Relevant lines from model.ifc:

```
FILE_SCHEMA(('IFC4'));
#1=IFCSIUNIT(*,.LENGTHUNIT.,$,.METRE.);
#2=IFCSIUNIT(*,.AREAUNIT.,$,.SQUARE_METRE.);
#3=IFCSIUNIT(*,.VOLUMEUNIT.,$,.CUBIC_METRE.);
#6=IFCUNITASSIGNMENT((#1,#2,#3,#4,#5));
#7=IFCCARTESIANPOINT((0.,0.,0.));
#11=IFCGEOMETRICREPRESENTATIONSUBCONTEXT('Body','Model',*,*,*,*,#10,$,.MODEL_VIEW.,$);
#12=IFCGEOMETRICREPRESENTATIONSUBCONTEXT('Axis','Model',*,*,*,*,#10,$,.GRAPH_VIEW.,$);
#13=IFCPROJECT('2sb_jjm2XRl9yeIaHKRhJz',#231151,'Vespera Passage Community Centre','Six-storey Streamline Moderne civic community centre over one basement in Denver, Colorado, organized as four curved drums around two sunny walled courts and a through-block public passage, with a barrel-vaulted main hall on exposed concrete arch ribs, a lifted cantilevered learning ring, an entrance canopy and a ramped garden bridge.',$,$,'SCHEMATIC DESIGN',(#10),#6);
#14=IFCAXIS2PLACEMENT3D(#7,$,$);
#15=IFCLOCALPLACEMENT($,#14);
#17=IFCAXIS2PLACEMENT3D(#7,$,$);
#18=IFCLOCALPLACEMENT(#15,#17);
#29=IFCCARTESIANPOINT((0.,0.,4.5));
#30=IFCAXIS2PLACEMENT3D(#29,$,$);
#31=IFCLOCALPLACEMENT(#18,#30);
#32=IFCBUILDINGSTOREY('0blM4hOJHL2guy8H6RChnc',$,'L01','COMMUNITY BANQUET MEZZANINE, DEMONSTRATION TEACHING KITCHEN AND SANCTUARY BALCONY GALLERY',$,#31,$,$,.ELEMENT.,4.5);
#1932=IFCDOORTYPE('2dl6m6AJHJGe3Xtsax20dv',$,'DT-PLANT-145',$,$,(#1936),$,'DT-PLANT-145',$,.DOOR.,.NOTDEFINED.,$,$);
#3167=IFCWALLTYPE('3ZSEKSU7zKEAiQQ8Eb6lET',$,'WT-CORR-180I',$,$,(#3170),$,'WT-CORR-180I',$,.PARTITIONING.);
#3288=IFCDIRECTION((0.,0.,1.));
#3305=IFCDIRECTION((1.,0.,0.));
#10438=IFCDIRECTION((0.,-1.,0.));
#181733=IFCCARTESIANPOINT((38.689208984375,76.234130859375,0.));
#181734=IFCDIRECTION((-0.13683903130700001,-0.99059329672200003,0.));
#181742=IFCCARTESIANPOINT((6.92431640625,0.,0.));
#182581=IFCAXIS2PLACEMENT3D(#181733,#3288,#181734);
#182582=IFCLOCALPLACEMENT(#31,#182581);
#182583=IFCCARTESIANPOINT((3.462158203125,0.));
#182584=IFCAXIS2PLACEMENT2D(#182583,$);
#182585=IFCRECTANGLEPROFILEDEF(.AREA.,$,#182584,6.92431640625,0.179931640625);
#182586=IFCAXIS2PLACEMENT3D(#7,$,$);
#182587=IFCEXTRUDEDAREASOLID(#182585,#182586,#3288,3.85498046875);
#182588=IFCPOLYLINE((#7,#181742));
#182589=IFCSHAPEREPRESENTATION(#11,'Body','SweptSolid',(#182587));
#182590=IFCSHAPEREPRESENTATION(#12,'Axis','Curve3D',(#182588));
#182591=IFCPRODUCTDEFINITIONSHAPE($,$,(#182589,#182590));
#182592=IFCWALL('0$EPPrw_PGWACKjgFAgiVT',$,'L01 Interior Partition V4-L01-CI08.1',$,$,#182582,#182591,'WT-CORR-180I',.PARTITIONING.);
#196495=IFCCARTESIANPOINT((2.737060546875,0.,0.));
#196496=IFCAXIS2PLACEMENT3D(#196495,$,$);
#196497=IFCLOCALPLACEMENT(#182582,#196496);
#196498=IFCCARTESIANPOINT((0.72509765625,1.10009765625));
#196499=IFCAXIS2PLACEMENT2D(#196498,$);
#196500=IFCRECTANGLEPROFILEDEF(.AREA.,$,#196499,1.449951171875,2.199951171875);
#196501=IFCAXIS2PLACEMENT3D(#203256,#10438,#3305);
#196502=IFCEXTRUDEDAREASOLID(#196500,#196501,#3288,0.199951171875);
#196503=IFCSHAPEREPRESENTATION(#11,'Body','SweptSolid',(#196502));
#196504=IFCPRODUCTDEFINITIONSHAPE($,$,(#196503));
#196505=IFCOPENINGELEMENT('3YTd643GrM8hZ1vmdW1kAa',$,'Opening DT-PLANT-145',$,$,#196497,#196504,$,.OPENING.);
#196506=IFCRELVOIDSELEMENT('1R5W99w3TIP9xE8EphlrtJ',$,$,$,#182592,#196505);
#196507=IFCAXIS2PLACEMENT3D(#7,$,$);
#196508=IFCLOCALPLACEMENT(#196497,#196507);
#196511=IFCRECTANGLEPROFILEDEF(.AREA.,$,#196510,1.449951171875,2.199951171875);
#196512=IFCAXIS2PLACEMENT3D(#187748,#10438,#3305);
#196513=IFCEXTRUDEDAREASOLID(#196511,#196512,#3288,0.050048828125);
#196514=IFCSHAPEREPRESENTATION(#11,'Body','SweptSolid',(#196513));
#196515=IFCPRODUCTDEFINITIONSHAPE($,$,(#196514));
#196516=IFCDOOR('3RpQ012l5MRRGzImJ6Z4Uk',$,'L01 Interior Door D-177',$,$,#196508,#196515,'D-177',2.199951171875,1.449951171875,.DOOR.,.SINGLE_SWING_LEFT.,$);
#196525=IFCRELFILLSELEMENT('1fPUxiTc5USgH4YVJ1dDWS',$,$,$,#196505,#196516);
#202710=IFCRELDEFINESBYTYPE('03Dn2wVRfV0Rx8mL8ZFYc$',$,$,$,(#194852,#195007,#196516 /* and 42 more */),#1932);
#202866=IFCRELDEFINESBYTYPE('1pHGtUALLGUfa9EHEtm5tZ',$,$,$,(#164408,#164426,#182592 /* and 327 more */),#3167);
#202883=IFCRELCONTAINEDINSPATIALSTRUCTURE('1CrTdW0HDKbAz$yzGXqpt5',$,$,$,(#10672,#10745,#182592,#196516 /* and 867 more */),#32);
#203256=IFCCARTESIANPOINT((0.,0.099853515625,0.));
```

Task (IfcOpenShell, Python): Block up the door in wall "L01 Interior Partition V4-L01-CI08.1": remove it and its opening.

```python
import ifcopenshell
import ifcopenshell.api.feature
import ifcopenshell.api.root
import ifcopenshell.geom
import ifcopenshell.util.shape

model = ifcopenshell.open("model.ifc")
settings = ifcopenshell.geom.settings()


def volume(element):
    """Net volume in cubic metres, openings subtracted."""
    shape = ifcopenshell.geom.create_shape(settings, element)
    return ifcopenshell.util.shape.get_volume(shape.geometry)


door = model.by_guid("3RpQ012l5MRRGzImJ6Z4Uk")
opening = door.FillsVoids[0].RelatingOpeningElement
wall = opening.VoidsElements[0].RelatingBuildingElement
before = volume(wall)

ifcopenshell.api.root.remove_product(model, product=door)
ifcopenshell.api.feature.remove_feature(model, feature=opening)

after = volume(wall)

print(f"wall volume {before:.3f} -> {after:.3f} m3")

model.write("model_rev.ifc")
```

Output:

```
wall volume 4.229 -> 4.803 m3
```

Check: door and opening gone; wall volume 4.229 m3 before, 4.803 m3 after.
